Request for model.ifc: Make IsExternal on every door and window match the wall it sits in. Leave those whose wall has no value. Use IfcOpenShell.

First a look at what the model holds.

```python
import ifcopenshell
import ifcopenshell.util.element

model = ifcopenshell.open("model.ifc")
print(model.schema)
seen = {}
for e in model.by_type("IfcDoor") + model.by_type("IfcWindow"):
    if not e.FillsVoids:
        continue
    host = e.FillsVoids[0].RelatingOpeningElement.VoidsElements[0].RelatingBuildingElement
    own = ifcopenshell.util.element.get_pset(e, f"Pset_{e.is_a()[3:].removesuffix('StandardCase')}Common", "IsExternal")
    wall = ifcopenshell.util.element.get_pset(host, "Pset_WallCommon", "IsExternal")
    seen[e.is_a(), own, wall] = seen.get((e.is_a(), own, wall), 0) + 1
for (cls, own, wall), count in sorted(seen.items(), key=str):
    print(count, cls, "IsExternal:", own, "| host wall:", wall)
```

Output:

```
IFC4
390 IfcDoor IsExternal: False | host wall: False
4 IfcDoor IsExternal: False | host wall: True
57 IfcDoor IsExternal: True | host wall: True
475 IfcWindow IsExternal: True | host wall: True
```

```python
import ifcopenshell
import ifcopenshell.api.pset
import ifcopenshell.util.element

model = ifcopenshell.open("model.ifc")

count = 0
for ifc_class, pset_name in (("IfcDoor", "Pset_DoorCommon"), ("IfcWindow", "Pset_WindowCommon")):
    for e in model.by_type(ifc_class):
        if not e.FillsVoids:
            continue
        host = e.FillsVoids[0].RelatingOpeningElement.VoidsElements[0].RelatingBuildingElement
        external = ifcopenshell.util.element.get_pset(host, "Pset_WallCommon", "IsExternal")
        if external is None or ifcopenshell.util.element.get_pset(e, pset_name, "IsExternal") == external:
            continue
        pset = ifcopenshell.api.pset.add_pset(model, product=e, name=pset_name)
        ifcopenshell.api.pset.edit_pset(model, pset=pset, properties={"IsExternal": external})
        count += 1

print(count, "updated")

model.write("model_updated.ifc")
```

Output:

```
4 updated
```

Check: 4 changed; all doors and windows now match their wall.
